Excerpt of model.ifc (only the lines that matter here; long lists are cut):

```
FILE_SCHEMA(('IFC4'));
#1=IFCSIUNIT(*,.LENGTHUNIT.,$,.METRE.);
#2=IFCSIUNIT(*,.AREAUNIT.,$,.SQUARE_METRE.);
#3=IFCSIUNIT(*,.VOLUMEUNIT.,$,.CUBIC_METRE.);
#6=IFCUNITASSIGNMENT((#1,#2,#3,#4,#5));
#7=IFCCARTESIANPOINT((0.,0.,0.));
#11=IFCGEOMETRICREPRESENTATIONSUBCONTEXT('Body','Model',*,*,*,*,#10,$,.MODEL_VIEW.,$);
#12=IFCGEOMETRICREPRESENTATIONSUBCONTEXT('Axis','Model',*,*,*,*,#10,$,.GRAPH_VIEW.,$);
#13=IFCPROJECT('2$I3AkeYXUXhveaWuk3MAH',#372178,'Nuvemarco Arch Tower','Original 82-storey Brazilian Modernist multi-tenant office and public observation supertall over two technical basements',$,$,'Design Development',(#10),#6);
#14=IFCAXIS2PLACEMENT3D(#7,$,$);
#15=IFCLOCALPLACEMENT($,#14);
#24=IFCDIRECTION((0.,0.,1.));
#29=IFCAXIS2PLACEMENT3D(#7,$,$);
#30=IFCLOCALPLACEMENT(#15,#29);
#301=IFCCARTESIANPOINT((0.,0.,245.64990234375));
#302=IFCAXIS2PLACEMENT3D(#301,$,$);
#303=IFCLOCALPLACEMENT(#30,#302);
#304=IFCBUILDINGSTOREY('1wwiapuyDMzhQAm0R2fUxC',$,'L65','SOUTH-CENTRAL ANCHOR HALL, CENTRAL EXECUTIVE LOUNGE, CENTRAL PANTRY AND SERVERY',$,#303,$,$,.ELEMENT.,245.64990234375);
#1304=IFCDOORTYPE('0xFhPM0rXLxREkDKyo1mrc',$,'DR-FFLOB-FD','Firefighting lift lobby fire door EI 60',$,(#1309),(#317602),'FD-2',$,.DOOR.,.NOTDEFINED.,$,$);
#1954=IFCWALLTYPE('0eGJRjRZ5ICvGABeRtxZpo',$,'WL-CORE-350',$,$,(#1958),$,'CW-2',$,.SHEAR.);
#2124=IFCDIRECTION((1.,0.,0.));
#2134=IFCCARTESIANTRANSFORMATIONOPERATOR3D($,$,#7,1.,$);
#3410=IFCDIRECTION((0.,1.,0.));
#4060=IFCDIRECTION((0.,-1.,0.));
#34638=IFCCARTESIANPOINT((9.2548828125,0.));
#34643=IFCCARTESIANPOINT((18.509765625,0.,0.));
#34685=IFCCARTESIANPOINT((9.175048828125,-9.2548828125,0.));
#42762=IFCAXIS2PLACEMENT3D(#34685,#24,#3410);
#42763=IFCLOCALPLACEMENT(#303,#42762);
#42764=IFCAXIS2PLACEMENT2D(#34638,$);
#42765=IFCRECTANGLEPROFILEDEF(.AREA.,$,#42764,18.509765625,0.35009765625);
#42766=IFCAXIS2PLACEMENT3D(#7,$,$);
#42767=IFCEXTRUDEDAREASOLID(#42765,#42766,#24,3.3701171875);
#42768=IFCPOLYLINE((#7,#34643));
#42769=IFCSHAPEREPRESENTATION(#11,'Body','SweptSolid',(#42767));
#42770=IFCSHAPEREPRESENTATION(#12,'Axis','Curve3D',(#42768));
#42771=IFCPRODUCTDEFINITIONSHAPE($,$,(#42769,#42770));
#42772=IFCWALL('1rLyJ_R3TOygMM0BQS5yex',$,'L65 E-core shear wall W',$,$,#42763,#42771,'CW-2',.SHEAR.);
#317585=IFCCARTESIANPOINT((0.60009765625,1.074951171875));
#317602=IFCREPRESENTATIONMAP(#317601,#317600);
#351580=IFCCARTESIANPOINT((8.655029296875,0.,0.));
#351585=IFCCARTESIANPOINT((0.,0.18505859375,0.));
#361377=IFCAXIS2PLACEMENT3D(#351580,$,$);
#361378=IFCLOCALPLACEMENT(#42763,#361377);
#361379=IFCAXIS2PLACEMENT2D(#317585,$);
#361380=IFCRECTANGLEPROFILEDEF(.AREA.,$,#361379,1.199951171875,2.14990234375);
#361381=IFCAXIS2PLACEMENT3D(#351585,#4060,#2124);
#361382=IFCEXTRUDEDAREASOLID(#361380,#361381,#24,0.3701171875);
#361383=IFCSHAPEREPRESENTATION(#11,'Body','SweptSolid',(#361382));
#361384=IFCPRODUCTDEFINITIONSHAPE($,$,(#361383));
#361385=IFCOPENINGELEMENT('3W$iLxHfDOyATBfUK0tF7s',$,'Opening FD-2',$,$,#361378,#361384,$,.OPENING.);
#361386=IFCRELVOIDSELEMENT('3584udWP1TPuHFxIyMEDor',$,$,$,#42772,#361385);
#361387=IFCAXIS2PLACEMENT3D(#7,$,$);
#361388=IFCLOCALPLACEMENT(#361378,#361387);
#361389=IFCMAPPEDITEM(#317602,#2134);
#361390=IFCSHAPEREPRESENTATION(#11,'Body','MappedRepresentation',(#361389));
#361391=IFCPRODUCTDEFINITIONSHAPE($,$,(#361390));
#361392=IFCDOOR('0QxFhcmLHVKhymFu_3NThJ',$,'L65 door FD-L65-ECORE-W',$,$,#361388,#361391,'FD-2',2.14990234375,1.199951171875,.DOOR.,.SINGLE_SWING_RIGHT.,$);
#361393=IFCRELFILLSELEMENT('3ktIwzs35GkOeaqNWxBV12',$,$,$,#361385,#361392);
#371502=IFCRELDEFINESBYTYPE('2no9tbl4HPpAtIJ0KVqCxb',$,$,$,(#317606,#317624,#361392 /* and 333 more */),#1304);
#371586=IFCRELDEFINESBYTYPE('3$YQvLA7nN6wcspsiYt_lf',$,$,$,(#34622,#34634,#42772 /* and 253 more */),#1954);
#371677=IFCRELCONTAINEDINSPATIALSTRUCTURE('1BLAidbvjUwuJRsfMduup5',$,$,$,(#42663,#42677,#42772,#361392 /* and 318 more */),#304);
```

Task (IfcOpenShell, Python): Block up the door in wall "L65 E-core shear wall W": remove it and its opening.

```python
import ifcopenshell
import ifcopenshell.api.feature
import ifcopenshell.api.root
import ifcopenshell.geom
import ifcopenshell.util.shape

model = ifcopenshell.open("model.ifc")
settings = ifcopenshell.geom.settings()


def volume(element):
    """Net volume in cubic metres, openings subtracted."""
    shape = ifcopenshell.geom.create_shape(settings, element)
    return ifcopenshell.util.shape.get_volume(shape.geometry)


door = model.by_guid("0QxFhcmLHVKhymFu_3NThJ")
opening = door.FillsVoids[0].RelatingOpeningElement
wall = opening.VoidsElements[0].RelatingBuildingElement
before = volume(wall)

ifcopenshell.api.root.remove_product(model, product=door)
ifcopenshell.api.feature.remove_feature(model, feature=opening)

after = volume(wall)

print(f"wall volume {before:.3f} -> {after:.3f} m3")

model.write("model_rev.ifc")
```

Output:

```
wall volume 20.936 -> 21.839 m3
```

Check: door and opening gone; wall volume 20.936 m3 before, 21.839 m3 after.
